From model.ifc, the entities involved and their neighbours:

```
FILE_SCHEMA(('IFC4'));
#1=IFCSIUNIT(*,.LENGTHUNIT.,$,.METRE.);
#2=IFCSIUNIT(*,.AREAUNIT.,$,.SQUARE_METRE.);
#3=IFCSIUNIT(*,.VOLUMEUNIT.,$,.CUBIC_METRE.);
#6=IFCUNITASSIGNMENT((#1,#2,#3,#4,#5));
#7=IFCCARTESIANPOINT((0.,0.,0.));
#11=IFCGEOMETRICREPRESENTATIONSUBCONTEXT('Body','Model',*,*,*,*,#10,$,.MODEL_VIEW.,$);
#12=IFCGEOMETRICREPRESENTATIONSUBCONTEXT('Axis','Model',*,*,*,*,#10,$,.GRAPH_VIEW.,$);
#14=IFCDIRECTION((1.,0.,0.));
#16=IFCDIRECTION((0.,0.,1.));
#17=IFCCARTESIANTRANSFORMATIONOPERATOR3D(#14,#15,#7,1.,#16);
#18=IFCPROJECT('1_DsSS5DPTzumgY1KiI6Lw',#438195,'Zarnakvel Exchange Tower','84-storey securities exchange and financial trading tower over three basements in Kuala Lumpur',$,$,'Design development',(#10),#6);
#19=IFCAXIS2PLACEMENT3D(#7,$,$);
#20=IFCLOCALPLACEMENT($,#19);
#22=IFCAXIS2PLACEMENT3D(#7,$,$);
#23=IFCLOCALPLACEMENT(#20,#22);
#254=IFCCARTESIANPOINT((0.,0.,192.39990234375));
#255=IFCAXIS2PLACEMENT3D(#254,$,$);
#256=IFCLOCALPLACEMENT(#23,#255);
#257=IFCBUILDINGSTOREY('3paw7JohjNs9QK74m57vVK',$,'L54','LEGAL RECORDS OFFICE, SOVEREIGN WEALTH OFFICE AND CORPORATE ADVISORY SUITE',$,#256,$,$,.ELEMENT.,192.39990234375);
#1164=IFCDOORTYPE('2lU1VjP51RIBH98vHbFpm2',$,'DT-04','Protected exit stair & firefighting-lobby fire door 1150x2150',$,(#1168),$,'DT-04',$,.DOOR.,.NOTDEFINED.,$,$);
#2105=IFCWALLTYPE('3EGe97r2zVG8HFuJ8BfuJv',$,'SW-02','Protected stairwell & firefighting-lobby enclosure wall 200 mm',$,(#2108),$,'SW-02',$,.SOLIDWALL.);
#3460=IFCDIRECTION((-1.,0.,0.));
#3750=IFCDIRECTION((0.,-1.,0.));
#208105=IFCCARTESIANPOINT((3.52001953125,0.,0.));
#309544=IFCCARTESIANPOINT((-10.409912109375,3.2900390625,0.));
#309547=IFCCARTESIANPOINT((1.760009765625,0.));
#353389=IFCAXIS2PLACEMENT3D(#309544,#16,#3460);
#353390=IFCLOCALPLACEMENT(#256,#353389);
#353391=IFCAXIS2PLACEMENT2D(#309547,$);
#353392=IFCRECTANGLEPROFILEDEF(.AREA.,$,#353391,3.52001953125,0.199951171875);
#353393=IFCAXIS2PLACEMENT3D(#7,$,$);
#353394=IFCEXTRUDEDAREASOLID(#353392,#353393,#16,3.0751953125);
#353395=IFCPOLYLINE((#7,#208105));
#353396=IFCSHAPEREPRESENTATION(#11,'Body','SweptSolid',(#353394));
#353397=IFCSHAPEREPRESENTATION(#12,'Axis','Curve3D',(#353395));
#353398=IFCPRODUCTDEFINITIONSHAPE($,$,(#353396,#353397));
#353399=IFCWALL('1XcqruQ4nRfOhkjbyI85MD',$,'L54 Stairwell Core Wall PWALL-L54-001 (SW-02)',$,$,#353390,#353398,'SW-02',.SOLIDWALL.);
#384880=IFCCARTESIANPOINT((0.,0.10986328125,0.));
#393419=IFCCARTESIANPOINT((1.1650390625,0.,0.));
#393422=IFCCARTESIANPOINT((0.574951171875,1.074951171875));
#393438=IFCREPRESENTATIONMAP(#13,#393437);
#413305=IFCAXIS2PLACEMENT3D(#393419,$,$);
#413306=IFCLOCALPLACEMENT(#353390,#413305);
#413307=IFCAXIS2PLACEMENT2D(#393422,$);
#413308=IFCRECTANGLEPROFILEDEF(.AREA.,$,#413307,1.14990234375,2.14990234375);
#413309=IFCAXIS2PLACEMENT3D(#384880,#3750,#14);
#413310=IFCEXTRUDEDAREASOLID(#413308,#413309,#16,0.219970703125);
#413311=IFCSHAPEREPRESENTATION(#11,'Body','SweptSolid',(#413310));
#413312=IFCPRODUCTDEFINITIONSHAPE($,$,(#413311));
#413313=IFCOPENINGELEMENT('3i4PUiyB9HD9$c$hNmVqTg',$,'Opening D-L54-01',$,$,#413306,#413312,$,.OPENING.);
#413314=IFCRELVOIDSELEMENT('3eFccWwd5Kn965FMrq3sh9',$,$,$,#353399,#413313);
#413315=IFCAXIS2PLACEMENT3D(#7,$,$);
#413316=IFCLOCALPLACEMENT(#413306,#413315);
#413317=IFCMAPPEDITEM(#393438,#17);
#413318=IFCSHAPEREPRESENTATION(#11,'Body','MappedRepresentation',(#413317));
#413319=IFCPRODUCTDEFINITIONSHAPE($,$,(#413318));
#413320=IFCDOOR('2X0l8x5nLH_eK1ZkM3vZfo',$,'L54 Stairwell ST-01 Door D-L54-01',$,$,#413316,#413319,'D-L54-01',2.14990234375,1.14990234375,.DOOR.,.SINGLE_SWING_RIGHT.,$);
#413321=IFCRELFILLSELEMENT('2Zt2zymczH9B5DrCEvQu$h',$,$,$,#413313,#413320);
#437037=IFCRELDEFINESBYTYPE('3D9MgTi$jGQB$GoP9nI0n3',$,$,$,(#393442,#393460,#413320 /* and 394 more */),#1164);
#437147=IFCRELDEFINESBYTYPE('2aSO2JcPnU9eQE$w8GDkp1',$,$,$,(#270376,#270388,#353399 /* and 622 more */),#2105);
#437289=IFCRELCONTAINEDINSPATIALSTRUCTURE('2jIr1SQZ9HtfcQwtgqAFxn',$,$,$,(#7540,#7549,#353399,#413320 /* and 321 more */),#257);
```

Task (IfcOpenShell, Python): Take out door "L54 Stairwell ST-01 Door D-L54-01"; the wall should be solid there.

```python
import ifcopenshell
import ifcopenshell.api.feature
import ifcopenshell.api.root
import ifcopenshell.geom
import ifcopenshell.util.shape

model = ifcopenshell.open("model.ifc")
settings = ifcopenshell.geom.settings()


def volume(element):
    """Net volume in cubic metres, openings subtracted."""
    shape = ifcopenshell.geom.create_shape(settings, element)
    return ifcopenshell.util.shape.get_volume(shape.geometry)


door = model.by_id(413320)
opening = door.FillsVoids[0].RelatingOpeningElement
wall = opening.VoidsElements[0].RelatingBuildingElement
before = volume(wall)

ifcopenshell.api.root.remove_product(model, product=door)
ifcopenshell.api.feature.remove_feature(model, feature=opening)

after = volume(wall)

print(f"wall volume {before:.3f} -> {after:.3f} m3")

model.write("model-out.ifc")
```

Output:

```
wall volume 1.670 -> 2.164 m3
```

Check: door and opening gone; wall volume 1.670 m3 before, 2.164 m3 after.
